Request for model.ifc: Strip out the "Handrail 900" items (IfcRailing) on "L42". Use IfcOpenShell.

First a look at what the model holds.

```python
import ifcopenshell
import ifcopenshell.util.element

model = ifcopenshell.open("model.ifc")
print(model.schema)
storey = next(s for s in model.by_type("IfcBuildingStorey") if s.Name == "L42")
railings = [e for e in ifcopenshell.util.element.get_decomposition(storey) if e.is_a("IfcRailing")]
seen = {}
for e in railings:
    element_type = ifcopenshell.util.element.get_type(e)
    name = element_type.Name if element_type not in (None, e) else None
    seen[name] = seen.get(name, 0) + 1
for name, count in sorted(seen.items(), key=str):
    print(count, "x", name)
```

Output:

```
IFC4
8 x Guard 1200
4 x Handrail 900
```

```python
import ifcopenshell
import ifcopenshell.api.root
import ifcopenshell.util.element

model = ifcopenshell.open("model.ifc")

storey = next(s for s in model.by_type("IfcBuildingStorey") if s.Name == "L42")
railings = [e for e in ifcopenshell.util.element.get_decomposition(storey) if e.is_a("IfcRailing")]
targets = [e for e in railings if (t := ifcopenshell.util.element.get_type(e)) not in (None, e) and t.Name == "Handrail 900"]

for e in targets:
    ifcopenshell.api.root.remove_product(model, product=e)
print(len(targets), "removed")

model.write("model_edited.ifc")
```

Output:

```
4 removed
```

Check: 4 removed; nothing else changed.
